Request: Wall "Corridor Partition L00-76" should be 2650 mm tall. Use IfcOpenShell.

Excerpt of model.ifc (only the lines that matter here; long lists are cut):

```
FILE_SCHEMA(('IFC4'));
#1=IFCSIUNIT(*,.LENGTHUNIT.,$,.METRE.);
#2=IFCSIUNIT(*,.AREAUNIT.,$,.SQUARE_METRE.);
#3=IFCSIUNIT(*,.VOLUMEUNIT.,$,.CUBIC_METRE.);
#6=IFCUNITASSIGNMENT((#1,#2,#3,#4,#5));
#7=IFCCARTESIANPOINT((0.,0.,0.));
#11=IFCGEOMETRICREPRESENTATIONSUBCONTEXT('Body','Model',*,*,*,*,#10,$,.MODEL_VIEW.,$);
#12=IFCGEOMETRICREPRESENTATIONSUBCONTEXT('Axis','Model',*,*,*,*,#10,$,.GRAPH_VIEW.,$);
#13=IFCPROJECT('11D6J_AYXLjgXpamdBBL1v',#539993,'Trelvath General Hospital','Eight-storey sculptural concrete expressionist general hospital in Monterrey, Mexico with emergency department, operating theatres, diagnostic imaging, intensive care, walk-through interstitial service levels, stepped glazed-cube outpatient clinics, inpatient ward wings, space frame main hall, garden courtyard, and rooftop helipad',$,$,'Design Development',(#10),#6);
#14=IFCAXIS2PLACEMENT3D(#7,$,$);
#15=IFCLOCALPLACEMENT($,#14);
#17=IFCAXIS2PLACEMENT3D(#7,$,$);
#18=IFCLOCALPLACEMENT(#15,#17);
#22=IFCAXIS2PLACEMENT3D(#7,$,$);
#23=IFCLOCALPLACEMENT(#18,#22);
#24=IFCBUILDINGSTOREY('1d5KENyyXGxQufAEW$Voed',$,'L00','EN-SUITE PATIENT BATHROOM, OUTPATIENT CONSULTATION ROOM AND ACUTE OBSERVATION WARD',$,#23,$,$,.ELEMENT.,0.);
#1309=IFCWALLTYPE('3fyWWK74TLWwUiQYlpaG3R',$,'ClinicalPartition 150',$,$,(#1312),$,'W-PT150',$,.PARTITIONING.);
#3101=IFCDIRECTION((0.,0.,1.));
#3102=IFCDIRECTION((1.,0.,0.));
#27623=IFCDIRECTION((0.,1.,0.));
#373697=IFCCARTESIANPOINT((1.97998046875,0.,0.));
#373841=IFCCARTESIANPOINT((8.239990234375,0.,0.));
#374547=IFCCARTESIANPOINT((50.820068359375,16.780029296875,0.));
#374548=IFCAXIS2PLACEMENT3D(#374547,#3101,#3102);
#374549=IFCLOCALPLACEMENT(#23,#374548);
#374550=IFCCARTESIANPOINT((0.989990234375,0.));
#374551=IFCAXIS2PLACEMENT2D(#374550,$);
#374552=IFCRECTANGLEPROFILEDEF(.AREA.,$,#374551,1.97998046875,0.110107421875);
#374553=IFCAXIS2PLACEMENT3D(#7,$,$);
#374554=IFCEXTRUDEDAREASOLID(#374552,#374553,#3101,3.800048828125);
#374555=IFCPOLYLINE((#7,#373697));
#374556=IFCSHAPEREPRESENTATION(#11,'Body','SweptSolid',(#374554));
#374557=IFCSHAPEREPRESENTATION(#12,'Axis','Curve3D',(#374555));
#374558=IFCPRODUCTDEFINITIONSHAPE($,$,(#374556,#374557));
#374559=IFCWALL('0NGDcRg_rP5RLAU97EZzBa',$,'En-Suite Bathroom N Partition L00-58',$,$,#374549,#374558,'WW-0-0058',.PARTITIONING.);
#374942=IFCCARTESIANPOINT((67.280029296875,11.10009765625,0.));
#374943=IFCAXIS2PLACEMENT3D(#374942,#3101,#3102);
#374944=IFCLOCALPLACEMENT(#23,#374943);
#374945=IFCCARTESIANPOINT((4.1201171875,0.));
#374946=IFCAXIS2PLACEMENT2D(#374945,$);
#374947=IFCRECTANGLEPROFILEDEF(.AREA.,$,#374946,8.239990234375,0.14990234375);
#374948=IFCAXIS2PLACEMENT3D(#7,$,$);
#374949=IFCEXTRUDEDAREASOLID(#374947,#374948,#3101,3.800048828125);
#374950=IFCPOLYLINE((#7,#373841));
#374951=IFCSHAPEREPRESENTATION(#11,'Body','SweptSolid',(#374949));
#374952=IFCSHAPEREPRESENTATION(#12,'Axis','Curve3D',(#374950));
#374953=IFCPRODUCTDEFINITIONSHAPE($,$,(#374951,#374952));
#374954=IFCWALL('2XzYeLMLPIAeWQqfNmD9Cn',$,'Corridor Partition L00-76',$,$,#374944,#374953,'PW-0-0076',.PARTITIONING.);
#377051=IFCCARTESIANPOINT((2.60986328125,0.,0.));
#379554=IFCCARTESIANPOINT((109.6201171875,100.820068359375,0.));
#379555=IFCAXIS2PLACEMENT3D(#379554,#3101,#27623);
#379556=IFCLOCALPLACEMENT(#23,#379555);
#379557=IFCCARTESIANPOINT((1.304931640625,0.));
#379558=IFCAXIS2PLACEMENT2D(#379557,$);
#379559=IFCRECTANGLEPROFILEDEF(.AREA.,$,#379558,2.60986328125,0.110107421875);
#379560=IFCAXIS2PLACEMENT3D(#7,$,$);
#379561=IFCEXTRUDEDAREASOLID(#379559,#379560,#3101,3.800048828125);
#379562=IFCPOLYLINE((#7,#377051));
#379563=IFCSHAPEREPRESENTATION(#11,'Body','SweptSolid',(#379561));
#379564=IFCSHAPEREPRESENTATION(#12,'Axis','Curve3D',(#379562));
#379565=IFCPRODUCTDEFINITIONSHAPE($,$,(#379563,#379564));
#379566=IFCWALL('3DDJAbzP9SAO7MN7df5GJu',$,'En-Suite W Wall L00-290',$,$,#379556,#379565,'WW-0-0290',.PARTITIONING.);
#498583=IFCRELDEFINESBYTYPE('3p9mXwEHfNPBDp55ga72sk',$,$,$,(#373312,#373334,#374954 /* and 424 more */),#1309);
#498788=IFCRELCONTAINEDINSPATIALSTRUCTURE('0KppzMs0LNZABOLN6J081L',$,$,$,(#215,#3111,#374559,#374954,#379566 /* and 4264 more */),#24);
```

```python
import ifcopenshell
import ifcopenshell.geom
import ifcopenshell.util.representation
import ifcopenshell.util.shape

model = ifcopenshell.open("model.ifc")
settings = ifcopenshell.geom.settings()


def volume(element):
    """Net volume in cubic metres, openings subtracted."""
    shape = ifcopenshell.geom.create_shape(settings, element)
    return ifcopenshell.util.shape.get_volume(shape.geometry)


wall = model.by_guid("2XzYeLMLPIAeWQqfNmD9Cn")
before = volume(wall)

body = ifcopenshell.util.representation.get_representation(wall, "Model", "Body")
solid = body.Items[0]
old_height = solid.Depth
solid.Depth = 2.65
after = volume(wall)

print(f"height {old_height:g} -> {solid.Depth:g}, volume {before:.3f} -> {after:.3f} m3")

model.write("model-out.ifc")
```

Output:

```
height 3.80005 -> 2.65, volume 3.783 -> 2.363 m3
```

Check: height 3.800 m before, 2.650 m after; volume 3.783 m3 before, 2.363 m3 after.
